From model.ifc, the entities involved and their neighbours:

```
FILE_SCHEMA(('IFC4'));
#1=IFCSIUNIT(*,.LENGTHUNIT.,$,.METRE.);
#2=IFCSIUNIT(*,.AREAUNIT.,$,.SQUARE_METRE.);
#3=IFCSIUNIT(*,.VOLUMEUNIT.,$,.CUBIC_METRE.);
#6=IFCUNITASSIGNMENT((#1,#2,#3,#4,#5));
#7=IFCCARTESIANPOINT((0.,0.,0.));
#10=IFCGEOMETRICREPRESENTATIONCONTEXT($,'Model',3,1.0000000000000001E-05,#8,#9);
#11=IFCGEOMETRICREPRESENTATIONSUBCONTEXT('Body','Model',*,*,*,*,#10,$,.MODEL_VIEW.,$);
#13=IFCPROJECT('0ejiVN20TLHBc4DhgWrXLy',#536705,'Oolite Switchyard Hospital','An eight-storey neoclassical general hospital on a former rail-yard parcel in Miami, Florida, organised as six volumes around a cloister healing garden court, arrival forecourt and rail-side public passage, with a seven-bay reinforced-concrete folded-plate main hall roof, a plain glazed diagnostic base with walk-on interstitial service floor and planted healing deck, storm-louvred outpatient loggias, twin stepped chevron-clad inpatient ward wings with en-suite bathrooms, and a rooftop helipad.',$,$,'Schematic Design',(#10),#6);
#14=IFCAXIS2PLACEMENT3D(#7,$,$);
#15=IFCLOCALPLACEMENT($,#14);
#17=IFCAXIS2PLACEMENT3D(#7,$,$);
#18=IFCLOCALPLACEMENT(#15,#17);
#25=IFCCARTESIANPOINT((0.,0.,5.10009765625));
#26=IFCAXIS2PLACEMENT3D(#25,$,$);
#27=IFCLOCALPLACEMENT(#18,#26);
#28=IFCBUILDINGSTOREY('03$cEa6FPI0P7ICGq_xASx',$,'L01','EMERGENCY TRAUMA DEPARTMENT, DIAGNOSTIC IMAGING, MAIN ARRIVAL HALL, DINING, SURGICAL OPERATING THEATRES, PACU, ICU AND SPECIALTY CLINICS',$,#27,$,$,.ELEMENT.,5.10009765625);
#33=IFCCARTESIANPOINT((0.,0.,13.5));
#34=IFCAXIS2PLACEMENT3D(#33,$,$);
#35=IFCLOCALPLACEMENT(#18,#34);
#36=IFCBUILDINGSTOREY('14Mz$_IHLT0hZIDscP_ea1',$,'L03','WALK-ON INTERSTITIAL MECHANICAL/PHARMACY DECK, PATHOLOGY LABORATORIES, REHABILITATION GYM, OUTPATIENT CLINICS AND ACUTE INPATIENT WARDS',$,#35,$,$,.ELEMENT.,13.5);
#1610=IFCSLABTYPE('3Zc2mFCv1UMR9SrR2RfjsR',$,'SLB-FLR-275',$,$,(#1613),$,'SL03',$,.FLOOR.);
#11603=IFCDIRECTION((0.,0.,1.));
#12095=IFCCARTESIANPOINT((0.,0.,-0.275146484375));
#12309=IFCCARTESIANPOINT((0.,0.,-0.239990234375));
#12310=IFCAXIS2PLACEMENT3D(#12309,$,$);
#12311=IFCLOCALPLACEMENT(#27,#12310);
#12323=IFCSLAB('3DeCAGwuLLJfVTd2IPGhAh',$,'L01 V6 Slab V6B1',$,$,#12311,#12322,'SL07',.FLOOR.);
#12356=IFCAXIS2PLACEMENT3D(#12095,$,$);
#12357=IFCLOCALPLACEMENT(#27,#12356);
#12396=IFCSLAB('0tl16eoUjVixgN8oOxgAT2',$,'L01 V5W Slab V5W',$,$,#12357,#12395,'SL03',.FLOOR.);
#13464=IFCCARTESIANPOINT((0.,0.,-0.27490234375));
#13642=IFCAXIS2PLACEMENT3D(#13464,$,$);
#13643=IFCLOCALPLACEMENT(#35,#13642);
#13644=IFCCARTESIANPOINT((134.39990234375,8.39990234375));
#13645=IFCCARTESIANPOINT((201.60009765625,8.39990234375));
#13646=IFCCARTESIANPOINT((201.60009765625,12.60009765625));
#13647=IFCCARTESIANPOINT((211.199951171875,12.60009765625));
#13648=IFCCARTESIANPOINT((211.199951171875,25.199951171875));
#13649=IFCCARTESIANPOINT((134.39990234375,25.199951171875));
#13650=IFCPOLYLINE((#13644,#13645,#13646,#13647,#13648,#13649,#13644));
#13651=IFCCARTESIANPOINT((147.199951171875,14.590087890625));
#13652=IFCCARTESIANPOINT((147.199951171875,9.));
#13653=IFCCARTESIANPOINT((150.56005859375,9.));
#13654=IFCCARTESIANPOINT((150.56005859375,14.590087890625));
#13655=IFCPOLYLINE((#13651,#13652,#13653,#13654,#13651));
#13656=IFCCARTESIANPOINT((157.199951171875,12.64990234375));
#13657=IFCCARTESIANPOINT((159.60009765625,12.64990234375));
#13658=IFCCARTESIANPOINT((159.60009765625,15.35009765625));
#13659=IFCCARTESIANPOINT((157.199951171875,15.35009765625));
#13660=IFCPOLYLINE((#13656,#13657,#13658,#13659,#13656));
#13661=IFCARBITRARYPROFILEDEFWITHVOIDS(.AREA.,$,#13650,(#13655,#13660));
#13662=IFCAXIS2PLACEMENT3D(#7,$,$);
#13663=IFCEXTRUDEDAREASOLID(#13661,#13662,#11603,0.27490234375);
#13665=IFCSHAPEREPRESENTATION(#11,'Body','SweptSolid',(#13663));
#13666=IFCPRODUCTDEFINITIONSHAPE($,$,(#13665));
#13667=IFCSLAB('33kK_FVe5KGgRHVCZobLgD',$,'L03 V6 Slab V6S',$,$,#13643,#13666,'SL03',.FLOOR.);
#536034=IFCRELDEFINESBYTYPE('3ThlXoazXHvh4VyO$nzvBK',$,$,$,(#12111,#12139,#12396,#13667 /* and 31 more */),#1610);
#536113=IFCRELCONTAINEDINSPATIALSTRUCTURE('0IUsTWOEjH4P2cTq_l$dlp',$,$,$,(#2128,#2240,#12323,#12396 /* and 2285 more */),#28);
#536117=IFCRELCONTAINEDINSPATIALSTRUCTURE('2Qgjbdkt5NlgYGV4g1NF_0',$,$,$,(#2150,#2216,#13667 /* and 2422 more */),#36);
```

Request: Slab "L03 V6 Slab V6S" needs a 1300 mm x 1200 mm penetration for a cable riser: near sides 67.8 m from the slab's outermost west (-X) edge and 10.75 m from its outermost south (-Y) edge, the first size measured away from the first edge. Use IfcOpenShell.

```python
import numpy as np
import ifcopenshell
import ifcopenshell.api.feature
import ifcopenshell.api.geometry
import ifcopenshell.api.root
import ifcopenshell.geom
import ifcopenshell.util.placement
import ifcopenshell.util.representation
import ifcopenshell.util.shape
import ifcopenshell.util.unit

model = ifcopenshell.open("model.ifc")
unit_scale = ifcopenshell.util.unit.calculate_unit_scale(model)
settings = ifcopenshell.geom.settings()


def volume(element):
    """Net volume in cubic metres, openings subtracted."""
    shape = ifcopenshell.geom.create_shape(settings, element)
    return ifcopenshell.util.shape.get_volume(shape.geometry)


slab = model.by_id(13667)
before = volume(slab)

# Extent in the slab's own axes, in metres. The edges named are its -X and -Y sides.
slab_shape = ifcopenshell.geom.create_shape(settings, slab)
vertices = ifcopenshell.util.shape.get_vertices(slab_shape.geometry)
x_min, y_min, bottom = vertices.min(axis=0)
top = vertices[:, 2].max()

opening = ifcopenshell.api.root.create_entity(model, ifc_class="IfcOpeningElement", name="Cable riser opening", predefined_type="OPENING")
context = ifcopenshell.util.representation.get_context(model, "Model", "Body", "MODEL_VIEW")
width, depth = 1.3, 1.2
outline = [(0.0, 0.0), (width, 0.0), (width, depth), (0.0, depth), (0.0, 0.0)]
# Overshoot both faces by 50 mm so the cut is clean.
shape = ifcopenshell.api.geometry.add_slab_representation(
    model, context=context, depth=top - bottom + 0.1, polyline=outline
)
ifcopenshell.api.geometry.assign_representation(model, product=opening, representation=shape)

matrix = ifcopenshell.util.placement.get_local_placement(slab.ObjectPlacement)
matrix[:, 3] = matrix @ np.append(np.array([x_min + 67.8, y_min + 10.75, bottom - 0.05]) / unit_scale, 1.0)
ifcopenshell.api.geometry.edit_object_placement(model, product=opening, matrix=matrix, is_si=False)
ifcopenshell.api.feature.add_feature(model, feature=opening, element=slab)

after = volume(slab)

print(f"slab volume {before:.3f} -> {after:.3f} m3")

model.write("model_updated.ifc")
```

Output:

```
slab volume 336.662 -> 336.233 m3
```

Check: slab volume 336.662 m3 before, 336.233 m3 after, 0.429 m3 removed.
